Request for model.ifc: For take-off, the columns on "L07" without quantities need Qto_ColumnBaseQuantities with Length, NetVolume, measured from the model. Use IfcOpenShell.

First a look at what the model holds.

```python
import ifcopenshell
import ifcopenshell.util.element
import ifcopenshell.util.unit

model = ifcopenshell.open("model.ifc")
print(model.schema)
for unit_type in ("LENGTHUNIT", "AREAUNIT", "VOLUMEUNIT"):
    print(unit_type, ifcopenshell.util.unit.calculate_unit_scale(model, unit_type))
storey = next(s for s in model.by_type("IfcBuildingStorey") if s.Name == "L07")
columns = [e for e in ifcopenshell.util.element.get_decomposition(storey) if e.is_a("IfcColumn")]
for e in sorted(columns, key=lambda e: e.id()):
    print(e.id(), e.is_a(), e.Name, list(ifcopenshell.util.element.get_psets(e, qtos_only=True)), sep=" | ")
```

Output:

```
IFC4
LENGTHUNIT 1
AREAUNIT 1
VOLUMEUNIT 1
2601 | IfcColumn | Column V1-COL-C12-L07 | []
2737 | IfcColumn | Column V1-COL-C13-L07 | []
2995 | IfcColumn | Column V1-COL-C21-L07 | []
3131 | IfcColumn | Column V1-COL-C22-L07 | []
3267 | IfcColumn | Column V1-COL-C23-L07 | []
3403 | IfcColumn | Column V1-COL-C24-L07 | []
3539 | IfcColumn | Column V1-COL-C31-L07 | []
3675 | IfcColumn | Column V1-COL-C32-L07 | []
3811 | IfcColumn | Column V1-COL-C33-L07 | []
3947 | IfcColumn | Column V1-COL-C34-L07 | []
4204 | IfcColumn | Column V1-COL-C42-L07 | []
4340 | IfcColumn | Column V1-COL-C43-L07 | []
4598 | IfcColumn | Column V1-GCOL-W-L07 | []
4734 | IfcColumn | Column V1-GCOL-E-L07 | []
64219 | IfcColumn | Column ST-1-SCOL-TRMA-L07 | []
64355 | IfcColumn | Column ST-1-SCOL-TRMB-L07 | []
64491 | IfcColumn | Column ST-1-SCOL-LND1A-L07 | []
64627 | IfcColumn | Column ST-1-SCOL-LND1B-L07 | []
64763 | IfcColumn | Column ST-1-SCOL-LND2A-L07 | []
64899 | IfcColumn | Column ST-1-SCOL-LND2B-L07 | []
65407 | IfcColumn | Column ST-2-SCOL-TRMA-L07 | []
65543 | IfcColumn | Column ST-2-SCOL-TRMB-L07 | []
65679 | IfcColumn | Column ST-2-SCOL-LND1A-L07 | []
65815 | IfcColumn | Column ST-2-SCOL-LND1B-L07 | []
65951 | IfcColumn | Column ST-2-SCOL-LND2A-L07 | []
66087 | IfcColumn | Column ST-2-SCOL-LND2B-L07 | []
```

```python
import ifcopenshell
import ifcopenshell.api.pset
import ifcopenshell.geom
import ifcopenshell.util.element
import ifcopenshell.util.shape
import ifcopenshell.util.unit

model = ifcopenshell.open("model.ifc")
unit_scale = ifcopenshell.util.unit.calculate_unit_scale(model)
volume_scale = ifcopenshell.util.unit.calculate_unit_scale(model, "VOLUMEUNIT")
settings = ifcopenshell.geom.settings()

storey = next(s for s in model.by_type("IfcBuildingStorey") if s.Name == "L07")
columns = [e for e in ifcopenshell.util.element.get_decomposition(storey) if e.is_a("IfcColumn")]

for e in sorted(columns, key=lambda e: e.id()):
    if ifcopenshell.util.element.get_psets(e, qtos_only=True, should_inherit=False):
        continue
    # Geometry comes back in metres, in the element's own axes.
    shape = ifcopenshell.geom.create_shape(settings, e)
    values = {
        "Length": ifcopenshell.util.shape.get_z(shape.geometry) / unit_scale,
        "NetVolume": ifcopenshell.util.shape.get_volume(shape.geometry) / volume_scale,
    }
    qto = ifcopenshell.api.pset.add_qto(model, product=e, name="Qto_ColumnBaseQuantities")
    ifcopenshell.api.pset.edit_qto(model, qto=qto, properties=values)
    print(e.id(), {k: round(v, 3) for k, v in values.items()})

model.write("model-out.ifc")
```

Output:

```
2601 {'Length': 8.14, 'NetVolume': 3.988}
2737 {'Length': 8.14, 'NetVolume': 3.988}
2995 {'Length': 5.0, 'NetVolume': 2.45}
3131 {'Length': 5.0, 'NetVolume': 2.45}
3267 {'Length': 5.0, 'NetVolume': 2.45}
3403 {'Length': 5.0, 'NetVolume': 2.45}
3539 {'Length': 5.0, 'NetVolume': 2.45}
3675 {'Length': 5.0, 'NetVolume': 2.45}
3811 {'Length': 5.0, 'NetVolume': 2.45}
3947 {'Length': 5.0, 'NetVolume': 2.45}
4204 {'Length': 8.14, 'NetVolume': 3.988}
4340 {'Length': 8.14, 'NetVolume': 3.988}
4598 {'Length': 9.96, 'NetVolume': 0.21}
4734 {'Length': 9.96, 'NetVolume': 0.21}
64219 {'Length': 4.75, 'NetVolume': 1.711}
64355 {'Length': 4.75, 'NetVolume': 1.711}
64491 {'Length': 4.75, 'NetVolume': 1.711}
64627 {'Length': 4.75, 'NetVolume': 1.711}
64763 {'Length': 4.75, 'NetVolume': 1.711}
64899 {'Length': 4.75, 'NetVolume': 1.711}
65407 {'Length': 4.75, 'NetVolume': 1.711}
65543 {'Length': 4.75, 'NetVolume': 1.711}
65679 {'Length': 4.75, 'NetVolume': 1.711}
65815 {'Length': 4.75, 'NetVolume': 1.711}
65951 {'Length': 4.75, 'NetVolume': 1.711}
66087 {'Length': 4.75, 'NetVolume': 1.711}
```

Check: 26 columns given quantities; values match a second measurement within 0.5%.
